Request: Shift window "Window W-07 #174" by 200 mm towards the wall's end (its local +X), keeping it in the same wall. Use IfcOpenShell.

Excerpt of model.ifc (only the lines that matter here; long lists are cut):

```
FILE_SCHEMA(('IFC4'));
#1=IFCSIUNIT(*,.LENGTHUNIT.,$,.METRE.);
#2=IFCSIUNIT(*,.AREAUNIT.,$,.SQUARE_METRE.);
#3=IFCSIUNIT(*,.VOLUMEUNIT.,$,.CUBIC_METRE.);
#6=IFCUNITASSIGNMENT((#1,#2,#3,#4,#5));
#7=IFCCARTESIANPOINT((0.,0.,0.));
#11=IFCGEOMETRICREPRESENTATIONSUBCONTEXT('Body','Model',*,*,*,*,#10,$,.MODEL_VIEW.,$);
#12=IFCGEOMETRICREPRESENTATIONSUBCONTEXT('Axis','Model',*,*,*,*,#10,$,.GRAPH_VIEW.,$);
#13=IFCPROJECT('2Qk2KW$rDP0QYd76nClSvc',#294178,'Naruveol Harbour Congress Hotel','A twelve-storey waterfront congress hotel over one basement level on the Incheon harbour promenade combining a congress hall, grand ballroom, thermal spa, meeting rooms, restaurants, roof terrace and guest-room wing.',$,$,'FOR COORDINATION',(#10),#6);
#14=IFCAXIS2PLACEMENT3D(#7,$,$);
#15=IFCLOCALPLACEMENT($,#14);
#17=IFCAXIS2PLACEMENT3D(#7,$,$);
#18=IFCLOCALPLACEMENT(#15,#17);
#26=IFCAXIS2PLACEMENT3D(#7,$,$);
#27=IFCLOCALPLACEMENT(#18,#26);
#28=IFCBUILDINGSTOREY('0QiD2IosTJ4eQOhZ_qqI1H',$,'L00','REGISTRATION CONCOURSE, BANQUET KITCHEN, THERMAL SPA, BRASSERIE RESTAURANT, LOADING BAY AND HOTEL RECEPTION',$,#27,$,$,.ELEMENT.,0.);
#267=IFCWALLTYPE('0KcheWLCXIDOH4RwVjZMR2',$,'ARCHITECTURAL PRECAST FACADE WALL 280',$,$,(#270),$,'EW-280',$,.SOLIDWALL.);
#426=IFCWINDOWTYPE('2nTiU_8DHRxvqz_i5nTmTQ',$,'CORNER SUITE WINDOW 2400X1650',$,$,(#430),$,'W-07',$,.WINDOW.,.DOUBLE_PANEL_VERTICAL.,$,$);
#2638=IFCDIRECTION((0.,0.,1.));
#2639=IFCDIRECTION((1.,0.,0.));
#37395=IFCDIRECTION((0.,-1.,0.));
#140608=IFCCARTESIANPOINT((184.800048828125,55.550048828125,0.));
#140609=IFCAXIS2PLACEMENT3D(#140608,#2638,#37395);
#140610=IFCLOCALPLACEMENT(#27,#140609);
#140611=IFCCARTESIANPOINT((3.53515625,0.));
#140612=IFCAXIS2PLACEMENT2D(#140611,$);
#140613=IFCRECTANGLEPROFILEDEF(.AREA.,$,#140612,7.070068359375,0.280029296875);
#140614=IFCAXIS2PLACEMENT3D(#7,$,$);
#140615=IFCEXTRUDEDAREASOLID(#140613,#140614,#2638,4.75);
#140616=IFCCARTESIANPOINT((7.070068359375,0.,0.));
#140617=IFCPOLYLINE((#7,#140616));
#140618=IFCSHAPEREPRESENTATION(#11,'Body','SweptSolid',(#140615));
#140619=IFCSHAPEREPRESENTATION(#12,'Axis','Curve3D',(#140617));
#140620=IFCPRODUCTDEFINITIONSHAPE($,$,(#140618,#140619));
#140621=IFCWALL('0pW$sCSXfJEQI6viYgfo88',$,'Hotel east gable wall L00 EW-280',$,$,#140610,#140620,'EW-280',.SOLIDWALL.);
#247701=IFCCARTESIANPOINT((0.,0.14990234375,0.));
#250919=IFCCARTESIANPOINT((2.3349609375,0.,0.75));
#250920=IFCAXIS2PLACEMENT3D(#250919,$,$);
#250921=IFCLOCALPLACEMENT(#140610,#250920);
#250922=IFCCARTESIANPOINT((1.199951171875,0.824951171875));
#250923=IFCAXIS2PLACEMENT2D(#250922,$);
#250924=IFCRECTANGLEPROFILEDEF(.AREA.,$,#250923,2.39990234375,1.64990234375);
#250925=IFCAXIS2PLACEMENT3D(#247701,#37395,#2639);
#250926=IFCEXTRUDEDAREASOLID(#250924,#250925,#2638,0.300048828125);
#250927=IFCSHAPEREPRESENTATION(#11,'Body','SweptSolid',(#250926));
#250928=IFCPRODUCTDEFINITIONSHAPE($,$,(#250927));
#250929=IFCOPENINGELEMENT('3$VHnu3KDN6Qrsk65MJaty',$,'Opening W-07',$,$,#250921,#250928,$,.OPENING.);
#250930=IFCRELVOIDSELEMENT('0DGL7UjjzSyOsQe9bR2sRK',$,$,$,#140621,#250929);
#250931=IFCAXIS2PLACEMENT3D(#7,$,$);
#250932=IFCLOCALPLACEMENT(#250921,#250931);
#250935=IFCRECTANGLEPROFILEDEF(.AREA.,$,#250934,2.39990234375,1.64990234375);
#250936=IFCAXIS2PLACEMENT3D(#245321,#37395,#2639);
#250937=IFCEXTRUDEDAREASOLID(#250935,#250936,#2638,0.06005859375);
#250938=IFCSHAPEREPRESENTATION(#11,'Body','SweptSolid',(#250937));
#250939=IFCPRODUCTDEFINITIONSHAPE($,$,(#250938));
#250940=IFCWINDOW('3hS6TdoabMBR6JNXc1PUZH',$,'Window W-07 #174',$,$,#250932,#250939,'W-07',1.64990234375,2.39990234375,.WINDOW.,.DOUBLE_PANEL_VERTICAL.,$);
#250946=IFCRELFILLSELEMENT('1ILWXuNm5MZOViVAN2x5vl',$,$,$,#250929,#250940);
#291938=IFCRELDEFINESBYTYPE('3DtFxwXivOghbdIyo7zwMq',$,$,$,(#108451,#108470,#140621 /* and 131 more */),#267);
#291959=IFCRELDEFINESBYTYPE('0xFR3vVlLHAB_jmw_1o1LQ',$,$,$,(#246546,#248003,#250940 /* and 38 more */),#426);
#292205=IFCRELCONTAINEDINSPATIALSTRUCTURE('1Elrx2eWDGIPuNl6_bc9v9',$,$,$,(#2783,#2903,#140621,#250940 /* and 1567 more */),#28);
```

```python
import ifcopenshell
import ifcopenshell.api.geometry
import ifcopenshell.util.placement

model = ifcopenshell.open("model.ifc")

window = model.by_guid("3hS6TdoabMBR6JNXc1PUZH")
opening = window.FillsVoids[0].RelatingOpeningElement
wall = opening.VoidsElements[0].RelatingBuildingElement

wall_matrix = ifcopenshell.util.placement.get_local_placement(wall.ObjectPlacement)
shift = wall_matrix[:3, 0] * 0.2
before = ifcopenshell.util.placement.get_local_placement(window.ObjectPlacement)[:3, 3].copy()

# The window is placed relative to its opening, so it follows when the opening moves.
matrix = ifcopenshell.util.placement.get_local_placement(opening.ObjectPlacement)
matrix[:3, 3] += shift
ifcopenshell.api.geometry.edit_object_placement(
    model, product=opening, matrix=matrix, is_si=False, should_transform_children=True
)

after = ifcopenshell.util.placement.get_local_placement(window.ObjectPlacement)[:3, 3]
print("window moved by", (after - before).round(3) + 0.0)

model.write("model_edited.ifc")
```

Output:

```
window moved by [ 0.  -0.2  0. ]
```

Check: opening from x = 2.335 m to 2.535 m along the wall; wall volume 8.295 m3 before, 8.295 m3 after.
